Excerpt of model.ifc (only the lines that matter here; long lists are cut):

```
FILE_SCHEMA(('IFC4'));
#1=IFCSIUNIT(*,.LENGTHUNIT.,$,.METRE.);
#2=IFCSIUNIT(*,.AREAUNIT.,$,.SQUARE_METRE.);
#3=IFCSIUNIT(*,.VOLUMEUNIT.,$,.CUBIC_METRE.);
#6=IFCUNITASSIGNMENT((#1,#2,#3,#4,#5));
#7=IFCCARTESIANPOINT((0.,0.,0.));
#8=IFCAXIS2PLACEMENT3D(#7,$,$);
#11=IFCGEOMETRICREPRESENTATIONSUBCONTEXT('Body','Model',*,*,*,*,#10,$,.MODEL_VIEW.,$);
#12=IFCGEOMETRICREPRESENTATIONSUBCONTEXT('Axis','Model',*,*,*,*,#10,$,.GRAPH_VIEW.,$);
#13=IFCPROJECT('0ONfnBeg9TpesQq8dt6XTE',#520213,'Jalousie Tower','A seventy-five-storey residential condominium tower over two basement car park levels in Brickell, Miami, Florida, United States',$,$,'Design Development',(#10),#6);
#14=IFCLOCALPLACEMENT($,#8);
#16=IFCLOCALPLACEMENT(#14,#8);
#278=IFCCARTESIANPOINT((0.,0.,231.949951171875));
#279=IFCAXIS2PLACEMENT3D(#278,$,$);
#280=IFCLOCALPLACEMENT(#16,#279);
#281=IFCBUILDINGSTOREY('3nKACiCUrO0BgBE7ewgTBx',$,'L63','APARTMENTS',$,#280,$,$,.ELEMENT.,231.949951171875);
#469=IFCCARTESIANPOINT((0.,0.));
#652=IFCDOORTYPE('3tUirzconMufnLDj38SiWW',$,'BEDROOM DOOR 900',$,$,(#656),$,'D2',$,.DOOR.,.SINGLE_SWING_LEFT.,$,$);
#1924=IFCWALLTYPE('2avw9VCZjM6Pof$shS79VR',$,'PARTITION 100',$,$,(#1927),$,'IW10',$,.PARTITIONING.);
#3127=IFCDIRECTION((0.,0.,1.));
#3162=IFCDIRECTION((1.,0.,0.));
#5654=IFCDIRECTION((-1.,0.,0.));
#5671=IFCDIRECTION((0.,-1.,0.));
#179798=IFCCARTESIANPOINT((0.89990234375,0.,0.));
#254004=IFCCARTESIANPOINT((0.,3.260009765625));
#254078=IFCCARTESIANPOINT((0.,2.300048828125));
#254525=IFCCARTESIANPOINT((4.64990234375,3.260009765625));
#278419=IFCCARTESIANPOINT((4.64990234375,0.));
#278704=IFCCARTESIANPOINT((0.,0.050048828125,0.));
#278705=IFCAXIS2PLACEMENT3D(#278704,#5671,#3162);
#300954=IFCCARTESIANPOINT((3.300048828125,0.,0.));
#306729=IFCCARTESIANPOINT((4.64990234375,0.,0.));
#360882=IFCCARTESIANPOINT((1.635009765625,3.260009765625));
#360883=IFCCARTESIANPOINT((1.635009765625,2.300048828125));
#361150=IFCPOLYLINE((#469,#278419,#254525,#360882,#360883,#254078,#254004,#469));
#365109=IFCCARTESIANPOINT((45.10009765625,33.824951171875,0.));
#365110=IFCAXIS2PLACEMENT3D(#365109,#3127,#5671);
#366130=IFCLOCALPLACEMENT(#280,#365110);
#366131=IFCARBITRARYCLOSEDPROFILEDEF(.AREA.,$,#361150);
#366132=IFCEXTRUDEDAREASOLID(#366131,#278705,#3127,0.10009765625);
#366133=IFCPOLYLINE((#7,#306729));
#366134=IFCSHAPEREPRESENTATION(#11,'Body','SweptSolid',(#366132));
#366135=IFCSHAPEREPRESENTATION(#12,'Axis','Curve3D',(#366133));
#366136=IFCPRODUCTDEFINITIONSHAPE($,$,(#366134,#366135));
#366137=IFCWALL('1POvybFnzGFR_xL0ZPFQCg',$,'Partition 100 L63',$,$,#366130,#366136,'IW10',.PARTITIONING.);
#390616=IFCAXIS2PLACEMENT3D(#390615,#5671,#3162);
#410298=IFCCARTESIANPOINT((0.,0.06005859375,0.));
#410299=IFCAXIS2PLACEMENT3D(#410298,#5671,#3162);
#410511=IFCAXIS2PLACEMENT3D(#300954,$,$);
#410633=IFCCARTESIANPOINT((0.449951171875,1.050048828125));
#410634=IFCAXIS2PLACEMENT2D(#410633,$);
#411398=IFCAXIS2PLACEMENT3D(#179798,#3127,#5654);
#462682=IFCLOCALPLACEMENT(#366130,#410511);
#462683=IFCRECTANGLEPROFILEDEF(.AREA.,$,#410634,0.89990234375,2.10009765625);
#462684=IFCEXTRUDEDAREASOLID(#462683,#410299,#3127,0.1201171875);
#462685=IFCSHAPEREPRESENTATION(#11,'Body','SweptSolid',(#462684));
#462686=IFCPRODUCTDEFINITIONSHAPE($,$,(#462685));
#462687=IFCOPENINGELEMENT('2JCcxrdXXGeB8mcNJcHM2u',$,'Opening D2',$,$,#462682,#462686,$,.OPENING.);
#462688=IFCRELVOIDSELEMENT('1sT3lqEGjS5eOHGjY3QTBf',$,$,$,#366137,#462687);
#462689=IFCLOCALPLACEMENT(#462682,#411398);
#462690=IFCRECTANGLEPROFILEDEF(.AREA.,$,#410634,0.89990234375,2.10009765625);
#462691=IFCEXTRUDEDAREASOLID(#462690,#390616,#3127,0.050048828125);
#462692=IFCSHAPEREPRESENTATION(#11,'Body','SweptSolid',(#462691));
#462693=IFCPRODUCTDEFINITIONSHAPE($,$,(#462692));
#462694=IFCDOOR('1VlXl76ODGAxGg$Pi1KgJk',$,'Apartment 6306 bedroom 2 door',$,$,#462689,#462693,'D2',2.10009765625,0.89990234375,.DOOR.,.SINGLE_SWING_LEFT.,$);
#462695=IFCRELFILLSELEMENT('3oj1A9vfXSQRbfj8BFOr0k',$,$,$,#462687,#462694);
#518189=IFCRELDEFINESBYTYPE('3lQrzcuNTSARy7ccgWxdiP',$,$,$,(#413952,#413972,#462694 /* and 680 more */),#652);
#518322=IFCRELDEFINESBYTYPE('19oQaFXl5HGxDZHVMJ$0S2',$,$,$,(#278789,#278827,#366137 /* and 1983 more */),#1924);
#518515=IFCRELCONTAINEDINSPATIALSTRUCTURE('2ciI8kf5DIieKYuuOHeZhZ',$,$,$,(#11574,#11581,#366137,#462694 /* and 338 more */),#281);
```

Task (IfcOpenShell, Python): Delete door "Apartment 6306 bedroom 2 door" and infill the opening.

```python
import ifcopenshell
import ifcopenshell.api.feature
import ifcopenshell.api.root
import ifcopenshell.geom
import ifcopenshell.util.shape

model = ifcopenshell.open("model.ifc")
settings = ifcopenshell.geom.settings()


def volume(element):
    """Net volume in cubic metres, openings subtracted."""
    shape = ifcopenshell.geom.create_shape(settings, element)
    return ifcopenshell.util.shape.get_volume(shape.geometry)


door = model.by_guid("1VlXl76ODGAxGg$Pi1KgJk")
opening = door.FillsVoids[0].RelatingOpeningElement
wall = opening.VoidsElements[0].RelatingBuildingElement
before = volume(wall)

ifcopenshell.api.root.remove_product(model, product=door)
ifcopenshell.api.feature.remove_feature(model, feature=opening)

after = volume(wall)

print(f"wall volume {before:.3f} -> {after:.3f} m3")

model.write("model-out.ifc")
```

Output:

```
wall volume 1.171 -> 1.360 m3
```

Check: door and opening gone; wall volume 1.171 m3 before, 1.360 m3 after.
